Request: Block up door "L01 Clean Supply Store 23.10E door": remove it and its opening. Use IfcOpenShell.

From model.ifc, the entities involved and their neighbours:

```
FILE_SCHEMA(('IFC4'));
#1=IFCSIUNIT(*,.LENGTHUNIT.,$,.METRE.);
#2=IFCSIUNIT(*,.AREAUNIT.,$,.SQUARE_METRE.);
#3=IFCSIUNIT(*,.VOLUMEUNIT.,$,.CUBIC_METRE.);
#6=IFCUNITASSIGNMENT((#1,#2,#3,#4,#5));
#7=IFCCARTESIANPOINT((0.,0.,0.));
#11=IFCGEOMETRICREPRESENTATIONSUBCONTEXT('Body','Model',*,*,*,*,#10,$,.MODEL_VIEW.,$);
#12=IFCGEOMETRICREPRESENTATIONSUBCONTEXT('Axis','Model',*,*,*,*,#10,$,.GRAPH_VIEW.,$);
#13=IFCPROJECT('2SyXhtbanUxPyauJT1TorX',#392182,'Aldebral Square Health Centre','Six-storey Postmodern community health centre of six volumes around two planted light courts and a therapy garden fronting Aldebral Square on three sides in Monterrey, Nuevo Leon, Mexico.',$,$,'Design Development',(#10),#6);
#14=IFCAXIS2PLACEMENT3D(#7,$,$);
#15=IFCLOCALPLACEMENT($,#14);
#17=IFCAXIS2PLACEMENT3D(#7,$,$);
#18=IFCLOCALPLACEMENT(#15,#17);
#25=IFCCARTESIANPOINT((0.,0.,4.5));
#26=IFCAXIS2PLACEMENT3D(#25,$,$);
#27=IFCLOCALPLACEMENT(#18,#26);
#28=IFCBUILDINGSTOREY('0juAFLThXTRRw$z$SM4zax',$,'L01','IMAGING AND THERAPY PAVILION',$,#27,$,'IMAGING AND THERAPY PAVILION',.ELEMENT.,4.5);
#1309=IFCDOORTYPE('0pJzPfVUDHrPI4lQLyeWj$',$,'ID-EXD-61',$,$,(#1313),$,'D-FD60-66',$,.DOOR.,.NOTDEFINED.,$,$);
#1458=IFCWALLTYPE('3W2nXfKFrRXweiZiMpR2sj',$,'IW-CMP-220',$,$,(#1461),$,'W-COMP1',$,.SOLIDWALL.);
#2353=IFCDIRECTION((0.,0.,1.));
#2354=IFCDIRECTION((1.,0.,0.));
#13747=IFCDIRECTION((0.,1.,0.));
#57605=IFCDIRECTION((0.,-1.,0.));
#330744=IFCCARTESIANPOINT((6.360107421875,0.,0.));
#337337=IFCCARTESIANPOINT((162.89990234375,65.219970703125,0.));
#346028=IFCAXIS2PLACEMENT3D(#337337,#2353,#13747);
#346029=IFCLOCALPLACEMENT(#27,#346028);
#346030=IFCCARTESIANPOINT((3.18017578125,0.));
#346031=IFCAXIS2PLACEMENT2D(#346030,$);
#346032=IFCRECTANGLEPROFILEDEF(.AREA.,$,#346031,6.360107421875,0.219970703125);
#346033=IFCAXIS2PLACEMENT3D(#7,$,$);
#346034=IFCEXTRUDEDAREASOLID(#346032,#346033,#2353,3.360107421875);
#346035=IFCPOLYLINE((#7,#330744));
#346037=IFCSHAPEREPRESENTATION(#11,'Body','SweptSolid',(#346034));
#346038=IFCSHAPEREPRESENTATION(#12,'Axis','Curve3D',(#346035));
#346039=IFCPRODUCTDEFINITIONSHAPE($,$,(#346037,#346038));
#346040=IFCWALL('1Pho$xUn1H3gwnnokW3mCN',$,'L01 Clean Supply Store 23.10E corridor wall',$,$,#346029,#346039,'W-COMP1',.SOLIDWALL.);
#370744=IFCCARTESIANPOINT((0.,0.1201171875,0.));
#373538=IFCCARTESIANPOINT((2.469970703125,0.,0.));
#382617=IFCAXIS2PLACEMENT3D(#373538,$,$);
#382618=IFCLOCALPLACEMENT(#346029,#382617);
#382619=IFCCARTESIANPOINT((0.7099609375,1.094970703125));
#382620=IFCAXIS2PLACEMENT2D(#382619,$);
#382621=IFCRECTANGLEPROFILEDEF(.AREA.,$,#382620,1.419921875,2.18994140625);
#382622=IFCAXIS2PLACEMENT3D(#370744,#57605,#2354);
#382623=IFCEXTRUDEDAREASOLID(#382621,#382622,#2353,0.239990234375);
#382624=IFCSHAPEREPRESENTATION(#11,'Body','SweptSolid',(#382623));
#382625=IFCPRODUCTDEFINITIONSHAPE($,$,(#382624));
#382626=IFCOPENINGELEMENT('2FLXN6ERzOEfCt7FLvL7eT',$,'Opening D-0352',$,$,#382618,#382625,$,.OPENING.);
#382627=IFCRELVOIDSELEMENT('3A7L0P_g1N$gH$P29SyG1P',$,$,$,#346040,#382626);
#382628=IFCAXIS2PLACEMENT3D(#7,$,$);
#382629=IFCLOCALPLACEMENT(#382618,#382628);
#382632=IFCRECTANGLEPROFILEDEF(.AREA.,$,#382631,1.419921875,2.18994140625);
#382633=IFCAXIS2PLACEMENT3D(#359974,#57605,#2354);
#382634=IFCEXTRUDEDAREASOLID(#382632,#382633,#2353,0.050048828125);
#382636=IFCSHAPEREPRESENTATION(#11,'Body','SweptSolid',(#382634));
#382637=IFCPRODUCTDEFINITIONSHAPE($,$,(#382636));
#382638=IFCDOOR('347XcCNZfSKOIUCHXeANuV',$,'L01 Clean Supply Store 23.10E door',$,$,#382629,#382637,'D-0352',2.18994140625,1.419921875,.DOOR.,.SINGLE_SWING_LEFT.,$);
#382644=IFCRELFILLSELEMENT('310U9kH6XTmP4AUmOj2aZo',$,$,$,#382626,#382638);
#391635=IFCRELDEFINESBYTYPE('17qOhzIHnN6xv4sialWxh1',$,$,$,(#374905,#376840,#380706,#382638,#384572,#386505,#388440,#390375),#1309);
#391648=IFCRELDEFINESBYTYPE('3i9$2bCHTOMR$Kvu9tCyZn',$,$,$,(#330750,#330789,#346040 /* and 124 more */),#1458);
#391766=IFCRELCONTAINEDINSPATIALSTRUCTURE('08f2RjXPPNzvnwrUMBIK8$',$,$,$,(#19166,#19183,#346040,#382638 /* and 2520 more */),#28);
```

```python
import ifcopenshell
import ifcopenshell.api.feature
import ifcopenshell.api.root
import ifcopenshell.geom
import ifcopenshell.util.shape

model = ifcopenshell.open("model.ifc")
settings = ifcopenshell.geom.settings()


def volume(element):
    """Net volume in cubic metres, openings subtracted."""
    shape = ifcopenshell.geom.create_shape(settings, element)
    return ifcopenshell.util.shape.get_volume(shape.geometry)


door = model.by_guid("347XcCNZfSKOIUCHXeANuV")
opening = door.FillsVoids[0].RelatingOpeningElement
wall = opening.VoidsElements[0].RelatingBuildingElement
before = volume(wall)

ifcopenshell.api.root.remove_product(model, product=door)
ifcopenshell.api.feature.remove_feature(model, feature=opening)

after = volume(wall)

print(f"wall volume {before:.3f} -> {after:.3f} m3")

model.write("model-out.ifc")
```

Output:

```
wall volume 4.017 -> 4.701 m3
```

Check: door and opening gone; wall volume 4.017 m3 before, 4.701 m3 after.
